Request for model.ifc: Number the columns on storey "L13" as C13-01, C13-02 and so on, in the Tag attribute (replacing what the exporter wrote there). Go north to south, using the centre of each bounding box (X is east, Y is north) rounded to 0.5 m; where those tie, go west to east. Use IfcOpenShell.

First a look at what the model holds.

```python
import ifcopenshell
import ifcopenshell.util.element
import ifcopenshell.util.placement

model = ifcopenshell.open("model.ifc")
print(model.schema)
storey = next(s for s in model.by_type("IfcBuildingStorey") if s.Name == "L13")
columns = [e for e in ifcopenshell.util.element.get_decomposition(storey) if e.is_a("IfcColumn")]
for e in sorted(columns, key=lambda e: e.id()):
    origin = ifcopenshell.util.placement.get_local_placement(e.ObjectPlacement)[:3, 3]
    print(e.id(), e.Tag, e.Name, origin.round(2) + 0.0, sep=" | ")
```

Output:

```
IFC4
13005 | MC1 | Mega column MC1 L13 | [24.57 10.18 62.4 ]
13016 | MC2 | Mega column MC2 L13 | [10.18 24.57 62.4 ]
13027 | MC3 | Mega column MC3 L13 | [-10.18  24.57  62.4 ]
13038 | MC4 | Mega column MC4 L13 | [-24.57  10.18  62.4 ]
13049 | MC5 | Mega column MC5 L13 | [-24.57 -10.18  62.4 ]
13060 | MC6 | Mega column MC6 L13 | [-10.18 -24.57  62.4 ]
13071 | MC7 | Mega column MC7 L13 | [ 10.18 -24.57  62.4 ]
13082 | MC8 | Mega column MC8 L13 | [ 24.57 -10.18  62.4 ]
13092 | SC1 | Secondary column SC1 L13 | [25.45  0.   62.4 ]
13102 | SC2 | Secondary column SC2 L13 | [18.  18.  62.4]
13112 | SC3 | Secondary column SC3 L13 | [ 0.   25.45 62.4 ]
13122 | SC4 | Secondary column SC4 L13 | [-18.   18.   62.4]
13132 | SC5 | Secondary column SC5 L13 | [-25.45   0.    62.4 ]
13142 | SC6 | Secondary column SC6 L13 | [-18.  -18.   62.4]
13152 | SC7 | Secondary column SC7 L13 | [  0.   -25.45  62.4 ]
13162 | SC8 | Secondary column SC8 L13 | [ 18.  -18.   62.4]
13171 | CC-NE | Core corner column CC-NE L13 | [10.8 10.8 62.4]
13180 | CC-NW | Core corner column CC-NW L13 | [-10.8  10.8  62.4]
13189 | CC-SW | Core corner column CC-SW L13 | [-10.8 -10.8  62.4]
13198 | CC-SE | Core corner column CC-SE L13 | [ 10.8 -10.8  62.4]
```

```python
import ifcopenshell
import ifcopenshell.geom
import ifcopenshell.util.element
import ifcopenshell.util.shape

model = ifcopenshell.open("model.ifc")
settings = ifcopenshell.geom.settings()
settings.set("use-world-coords", True)


def centre(element):
    shape = ifcopenshell.geom.create_shape(settings, element)
    return ifcopenshell.util.shape.get_bbox_centroid(shape.geometry)


storey = next(s for s in model.by_type("IfcBuildingStorey") if s.Name == "L13")
columns = [e for e in ifcopenshell.util.element.get_decomposition(storey) if e.is_a("IfcColumn")]

# Insertion points can sit at a corner or the storey origin, so sort by the geometry (in metres).
centres = {e: centre(e) for e in columns}
columns.sort(key=lambda e: (-round(centres[e][1] / 0.5), centres[e][0]))

for i, e in enumerate(columns, start=1):
    number = f"C13-{i:02d}"
    e.Tag = number
    print(e.id(), number)

model.write("model_v2.ifc")
```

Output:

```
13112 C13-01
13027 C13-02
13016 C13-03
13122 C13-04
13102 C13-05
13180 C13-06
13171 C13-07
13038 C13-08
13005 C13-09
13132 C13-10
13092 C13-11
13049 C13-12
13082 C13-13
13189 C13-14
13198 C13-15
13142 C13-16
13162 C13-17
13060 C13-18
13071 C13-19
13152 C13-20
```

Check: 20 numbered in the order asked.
